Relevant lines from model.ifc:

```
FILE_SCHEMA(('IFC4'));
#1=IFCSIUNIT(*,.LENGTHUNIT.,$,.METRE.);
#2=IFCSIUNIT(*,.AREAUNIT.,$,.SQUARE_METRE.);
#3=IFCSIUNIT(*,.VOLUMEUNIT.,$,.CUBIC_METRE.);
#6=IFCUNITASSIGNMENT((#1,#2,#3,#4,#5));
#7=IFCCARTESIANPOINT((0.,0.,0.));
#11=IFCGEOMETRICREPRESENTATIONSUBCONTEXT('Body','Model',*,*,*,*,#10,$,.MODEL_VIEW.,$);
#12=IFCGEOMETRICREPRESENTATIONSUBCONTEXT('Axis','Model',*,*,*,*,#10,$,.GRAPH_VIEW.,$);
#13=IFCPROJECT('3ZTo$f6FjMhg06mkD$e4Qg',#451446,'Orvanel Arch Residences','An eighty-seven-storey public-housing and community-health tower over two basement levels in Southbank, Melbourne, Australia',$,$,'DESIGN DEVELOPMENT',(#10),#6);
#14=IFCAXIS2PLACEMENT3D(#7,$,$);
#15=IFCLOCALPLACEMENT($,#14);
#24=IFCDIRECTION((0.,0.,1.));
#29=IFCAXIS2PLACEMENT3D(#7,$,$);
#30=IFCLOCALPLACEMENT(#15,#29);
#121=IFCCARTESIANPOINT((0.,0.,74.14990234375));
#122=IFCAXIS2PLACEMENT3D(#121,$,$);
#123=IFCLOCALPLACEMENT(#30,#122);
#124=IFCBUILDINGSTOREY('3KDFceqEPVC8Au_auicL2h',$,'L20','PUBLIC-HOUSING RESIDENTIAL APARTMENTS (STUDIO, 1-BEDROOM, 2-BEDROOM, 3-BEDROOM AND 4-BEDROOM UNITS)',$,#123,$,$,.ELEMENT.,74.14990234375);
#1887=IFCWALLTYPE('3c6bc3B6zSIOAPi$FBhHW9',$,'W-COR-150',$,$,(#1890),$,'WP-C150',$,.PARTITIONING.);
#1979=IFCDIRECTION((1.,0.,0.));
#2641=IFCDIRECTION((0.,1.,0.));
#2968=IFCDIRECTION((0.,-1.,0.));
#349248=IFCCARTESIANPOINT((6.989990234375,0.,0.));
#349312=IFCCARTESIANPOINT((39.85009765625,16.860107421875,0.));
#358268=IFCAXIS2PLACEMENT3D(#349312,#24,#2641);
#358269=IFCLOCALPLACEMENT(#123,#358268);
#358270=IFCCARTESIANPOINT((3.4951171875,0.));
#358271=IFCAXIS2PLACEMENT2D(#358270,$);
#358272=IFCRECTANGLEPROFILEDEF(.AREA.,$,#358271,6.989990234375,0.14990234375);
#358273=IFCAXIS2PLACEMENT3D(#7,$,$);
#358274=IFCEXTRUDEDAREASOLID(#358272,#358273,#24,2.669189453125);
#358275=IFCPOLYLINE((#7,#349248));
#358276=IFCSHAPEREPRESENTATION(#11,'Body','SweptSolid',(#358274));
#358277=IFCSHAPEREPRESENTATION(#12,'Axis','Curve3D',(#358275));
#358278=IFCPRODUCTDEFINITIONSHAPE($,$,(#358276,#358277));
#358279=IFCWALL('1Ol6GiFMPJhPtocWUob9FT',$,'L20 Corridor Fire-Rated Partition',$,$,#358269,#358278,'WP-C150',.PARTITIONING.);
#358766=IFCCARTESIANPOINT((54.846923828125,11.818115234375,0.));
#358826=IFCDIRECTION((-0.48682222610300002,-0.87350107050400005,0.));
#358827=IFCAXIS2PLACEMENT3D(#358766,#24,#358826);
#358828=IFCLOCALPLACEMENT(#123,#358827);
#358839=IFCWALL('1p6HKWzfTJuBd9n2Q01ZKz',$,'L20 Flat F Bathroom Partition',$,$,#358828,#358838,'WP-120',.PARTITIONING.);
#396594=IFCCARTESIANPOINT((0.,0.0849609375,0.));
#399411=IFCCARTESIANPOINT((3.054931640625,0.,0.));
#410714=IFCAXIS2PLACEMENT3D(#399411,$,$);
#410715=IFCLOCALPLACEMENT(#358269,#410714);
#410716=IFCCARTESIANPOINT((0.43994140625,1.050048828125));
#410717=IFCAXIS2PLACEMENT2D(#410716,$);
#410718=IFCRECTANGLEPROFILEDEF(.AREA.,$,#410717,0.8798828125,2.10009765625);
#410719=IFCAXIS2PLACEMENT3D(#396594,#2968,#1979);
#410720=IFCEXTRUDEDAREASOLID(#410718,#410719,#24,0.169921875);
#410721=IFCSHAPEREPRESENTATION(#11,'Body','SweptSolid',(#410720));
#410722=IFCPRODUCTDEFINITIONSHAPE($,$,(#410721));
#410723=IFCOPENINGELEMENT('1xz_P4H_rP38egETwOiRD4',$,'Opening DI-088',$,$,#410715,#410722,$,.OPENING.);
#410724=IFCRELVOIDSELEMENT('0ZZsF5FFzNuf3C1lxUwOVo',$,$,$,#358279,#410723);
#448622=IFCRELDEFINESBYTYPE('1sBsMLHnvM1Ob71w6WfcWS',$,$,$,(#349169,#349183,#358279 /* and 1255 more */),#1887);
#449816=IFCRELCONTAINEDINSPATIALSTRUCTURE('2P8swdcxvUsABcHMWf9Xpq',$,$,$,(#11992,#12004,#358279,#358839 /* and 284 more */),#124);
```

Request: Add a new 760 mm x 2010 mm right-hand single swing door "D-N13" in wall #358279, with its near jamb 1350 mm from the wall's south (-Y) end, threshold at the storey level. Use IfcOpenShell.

```python
import numpy as np
import ifcopenshell
import ifcopenshell.api.feature
import ifcopenshell.api.geometry
import ifcopenshell.api.root
import ifcopenshell.api.spatial
import ifcopenshell.geom
import ifcopenshell.util.element
import ifcopenshell.util.placement
import ifcopenshell.util.representation
import ifcopenshell.util.shape
import ifcopenshell.util.unit

model = ifcopenshell.open("model.ifc")
unit_scale = ifcopenshell.util.unit.calculate_unit_scale(model)
settings = ifcopenshell.geom.settings()


def volume(element):
    """Net volume in cubic metres, openings subtracted."""
    shape = ifcopenshell.geom.create_shape(settings, element)
    return ifcopenshell.util.shape.get_volume(shape.geometry)


wall = model.by_guid("1Ol6GiFMPJhPtocWUob9FT")
storey = ifcopenshell.util.element.get_container(wall, ifc_class="IfcBuildingStorey")
context = ifcopenshell.util.representation.get_context(model, "Model", "Body", "MODEL_VIEW")
before = volume(wall)

width, height, from_end, sill = 0.76, 2.01, 1.35, 0.0  # metres

# The wall runs along its own X axis, and the end named is its -X end.
wall_shape = ifcopenshell.geom.create_shape(settings, wall)
x, y, z = ifcopenshell.util.shape.get_vertices(wall_shape.geometry).T
start = x.min() + from_end
face, thickness = float(y.min()), float(y.max() - y.min())
wall_matrix = ifcopenshell.util.placement.get_local_placement(wall.ObjectPlacement)
level = ifcopenshell.util.placement.get_local_placement(storey.ObjectPlacement)[2, 3]


def in_wall(x, y):
    """Placement at x, y metres in the wall's axes, at sill height."""
    matrix = wall_matrix.copy()
    matrix[:, 3] = wall_matrix @ np.array([x / unit_scale, y / unit_scale, 0.0, 1.0])
    matrix[2, 3] = level + sill / unit_scale
    return matrix


# Opening: a box that overshoots both wall faces by 50 mm.
opening = ifcopenshell.api.root.create_entity(model, ifc_class="IfcOpeningElement", predefined_type="OPENING")
box = ifcopenshell.api.geometry.add_wall_representation(
    model, context=context, length=width, height=height, thickness=thickness + 0.1
)
ifcopenshell.api.geometry.assign_representation(model, product=opening, representation=box)
ifcopenshell.api.geometry.edit_object_placement(model, product=opening, matrix=in_wall(start, face - 0.05), is_si=False)
ifcopenshell.api.feature.add_feature(model, feature=opening, element=wall)

door = ifcopenshell.api.root.create_entity(model, ifc_class="IfcDoor", name="D-N13", predefined_type="DOOR")
door.OverallWidth, door.OverallHeight = width / unit_scale, height / unit_scale
door.OperationType = "SINGLE_SWING_RIGHT"
body = ifcopenshell.api.geometry.add_door_representation(
    model,
    context=context,
    overall_width=door.OverallWidth,
    overall_height=door.OverallHeight,
    operation_type="SINGLE_SWING_RIGHT",
    lining_properties={"LiningDepth": thickness / unit_scale, "ThresholdDepth": thickness / unit_scale},
)
ifcopenshell.api.geometry.assign_representation(model, product=door, representation=body)
ifcopenshell.api.spatial.assign_container(model, products=[door], relating_structure=storey)
ifcopenshell.api.feature.add_filling(model, opening=opening, element=door)

# The lining spans the wall, so the door starts at the wall face.
ifcopenshell.api.geometry.edit_object_placement(model, product=door, matrix=in_wall(start, face), is_si=False)

after = volume(wall)

print(f"wall volume {before:.3f} -> {after:.3f} m3")

model.write("model_updated.ifc")
```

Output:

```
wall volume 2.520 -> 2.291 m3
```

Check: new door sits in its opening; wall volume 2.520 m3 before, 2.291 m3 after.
